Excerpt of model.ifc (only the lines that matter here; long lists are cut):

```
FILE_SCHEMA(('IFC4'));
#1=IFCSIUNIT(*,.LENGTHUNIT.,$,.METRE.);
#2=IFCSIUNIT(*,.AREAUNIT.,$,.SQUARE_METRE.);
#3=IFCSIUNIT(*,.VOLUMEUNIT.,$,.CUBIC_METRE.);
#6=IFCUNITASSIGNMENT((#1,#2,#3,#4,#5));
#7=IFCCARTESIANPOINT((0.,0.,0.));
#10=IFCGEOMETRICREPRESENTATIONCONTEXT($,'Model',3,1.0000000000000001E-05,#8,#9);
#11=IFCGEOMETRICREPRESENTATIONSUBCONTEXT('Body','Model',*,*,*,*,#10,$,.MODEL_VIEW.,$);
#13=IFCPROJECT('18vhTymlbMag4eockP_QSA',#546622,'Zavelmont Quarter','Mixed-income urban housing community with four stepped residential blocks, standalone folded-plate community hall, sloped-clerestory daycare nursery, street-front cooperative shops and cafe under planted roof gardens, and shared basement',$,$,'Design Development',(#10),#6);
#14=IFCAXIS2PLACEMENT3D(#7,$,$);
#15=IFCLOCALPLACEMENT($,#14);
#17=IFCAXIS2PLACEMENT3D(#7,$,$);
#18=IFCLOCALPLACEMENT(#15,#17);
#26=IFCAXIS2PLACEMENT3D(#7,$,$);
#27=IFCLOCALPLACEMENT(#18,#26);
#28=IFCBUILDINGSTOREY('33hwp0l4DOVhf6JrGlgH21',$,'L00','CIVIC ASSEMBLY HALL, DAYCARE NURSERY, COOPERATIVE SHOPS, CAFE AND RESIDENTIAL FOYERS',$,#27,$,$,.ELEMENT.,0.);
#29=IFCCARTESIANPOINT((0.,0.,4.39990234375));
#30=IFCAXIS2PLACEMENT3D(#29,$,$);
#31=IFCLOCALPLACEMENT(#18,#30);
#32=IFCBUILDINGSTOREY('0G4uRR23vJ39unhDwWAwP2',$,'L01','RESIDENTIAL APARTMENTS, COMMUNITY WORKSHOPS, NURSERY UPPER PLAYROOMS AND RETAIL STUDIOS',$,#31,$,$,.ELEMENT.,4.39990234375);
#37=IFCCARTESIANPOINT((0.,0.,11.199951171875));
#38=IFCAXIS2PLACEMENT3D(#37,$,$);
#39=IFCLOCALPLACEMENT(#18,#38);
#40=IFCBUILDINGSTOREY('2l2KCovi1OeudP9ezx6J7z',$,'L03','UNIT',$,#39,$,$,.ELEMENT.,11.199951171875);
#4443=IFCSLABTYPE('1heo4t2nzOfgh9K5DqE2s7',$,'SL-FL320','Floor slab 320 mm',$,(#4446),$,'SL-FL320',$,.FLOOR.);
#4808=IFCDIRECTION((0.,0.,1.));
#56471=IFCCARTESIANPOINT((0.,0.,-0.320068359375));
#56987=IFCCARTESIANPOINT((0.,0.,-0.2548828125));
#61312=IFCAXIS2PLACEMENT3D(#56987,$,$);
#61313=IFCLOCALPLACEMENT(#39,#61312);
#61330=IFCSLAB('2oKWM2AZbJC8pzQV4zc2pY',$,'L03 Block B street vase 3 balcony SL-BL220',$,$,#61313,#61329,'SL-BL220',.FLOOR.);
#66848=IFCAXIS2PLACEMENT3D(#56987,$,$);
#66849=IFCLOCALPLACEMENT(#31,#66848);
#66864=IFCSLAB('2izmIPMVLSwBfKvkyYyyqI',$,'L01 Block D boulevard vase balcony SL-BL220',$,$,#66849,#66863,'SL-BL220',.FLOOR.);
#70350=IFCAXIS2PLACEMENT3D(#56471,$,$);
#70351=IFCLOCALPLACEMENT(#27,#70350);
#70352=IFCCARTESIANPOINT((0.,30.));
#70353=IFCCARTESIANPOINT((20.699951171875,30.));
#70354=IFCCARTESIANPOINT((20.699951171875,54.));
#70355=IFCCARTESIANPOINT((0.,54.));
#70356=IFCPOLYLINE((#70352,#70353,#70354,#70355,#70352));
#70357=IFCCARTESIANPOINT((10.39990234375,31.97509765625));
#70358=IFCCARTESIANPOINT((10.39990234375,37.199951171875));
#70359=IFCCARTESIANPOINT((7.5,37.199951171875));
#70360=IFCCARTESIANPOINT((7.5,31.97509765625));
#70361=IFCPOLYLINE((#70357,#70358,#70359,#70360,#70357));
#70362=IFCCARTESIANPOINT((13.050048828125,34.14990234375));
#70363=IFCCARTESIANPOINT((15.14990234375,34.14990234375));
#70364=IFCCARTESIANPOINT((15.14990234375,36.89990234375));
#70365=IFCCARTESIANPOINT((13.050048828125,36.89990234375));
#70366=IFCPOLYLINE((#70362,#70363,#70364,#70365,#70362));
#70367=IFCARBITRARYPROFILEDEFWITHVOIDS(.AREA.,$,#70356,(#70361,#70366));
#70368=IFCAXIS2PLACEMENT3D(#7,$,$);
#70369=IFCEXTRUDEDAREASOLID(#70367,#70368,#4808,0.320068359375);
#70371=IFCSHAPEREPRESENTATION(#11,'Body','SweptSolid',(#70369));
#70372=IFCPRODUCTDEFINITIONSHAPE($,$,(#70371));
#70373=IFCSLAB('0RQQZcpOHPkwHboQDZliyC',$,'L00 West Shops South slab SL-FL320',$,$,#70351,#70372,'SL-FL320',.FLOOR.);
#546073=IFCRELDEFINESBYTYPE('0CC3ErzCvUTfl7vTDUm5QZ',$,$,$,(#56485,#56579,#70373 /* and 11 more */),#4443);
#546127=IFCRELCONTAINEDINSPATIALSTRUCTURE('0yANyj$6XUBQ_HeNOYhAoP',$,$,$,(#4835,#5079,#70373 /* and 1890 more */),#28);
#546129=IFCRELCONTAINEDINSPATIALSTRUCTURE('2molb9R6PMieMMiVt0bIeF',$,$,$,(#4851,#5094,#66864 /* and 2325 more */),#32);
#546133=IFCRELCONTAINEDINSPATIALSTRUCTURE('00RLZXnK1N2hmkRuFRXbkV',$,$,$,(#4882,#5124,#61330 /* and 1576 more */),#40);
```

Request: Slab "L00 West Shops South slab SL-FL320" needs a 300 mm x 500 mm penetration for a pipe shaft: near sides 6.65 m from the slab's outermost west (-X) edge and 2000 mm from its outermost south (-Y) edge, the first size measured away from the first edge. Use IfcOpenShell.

```python
import numpy as np
import ifcopenshell
import ifcopenshell.api.feature
import ifcopenshell.api.geometry
import ifcopenshell.api.root
import ifcopenshell.geom
import ifcopenshell.util.placement
import ifcopenshell.util.representation
import ifcopenshell.util.shape
import ifcopenshell.util.unit

model = ifcopenshell.open("model.ifc")
unit_scale = ifcopenshell.util.unit.calculate_unit_scale(model)
settings = ifcopenshell.geom.settings()


def volume(element):
    """Net volume in cubic metres, openings subtracted."""
    shape = ifcopenshell.geom.create_shape(settings, element)
    return ifcopenshell.util.shape.get_volume(shape.geometry)


slab = model.by_guid("0RQQZcpOHPkwHboQDZliyC")
before = volume(slab)

# Extent in the slab's own axes, in metres. The edges named are its -X and -Y sides.
slab_shape = ifcopenshell.geom.create_shape(settings, slab)
vertices = ifcopenshell.util.shape.get_vertices(slab_shape.geometry)
x_min, y_min, bottom = vertices.min(axis=0)
top = vertices[:, 2].max()

opening = ifcopenshell.api.root.create_entity(model, ifc_class="IfcOpeningElement", name="Pipe shaft opening", predefined_type="OPENING")
context = ifcopenshell.util.representation.get_context(model, "Model", "Body", "MODEL_VIEW")
width, depth = 0.3, 0.5
outline = [(0.0, 0.0), (width, 0.0), (width, depth), (0.0, depth), (0.0, 0.0)]
# Overshoot both faces by 50 mm so the cut is clean.
shape = ifcopenshell.api.geometry.add_slab_representation(
    model, context=context, depth=top - bottom + 0.1, polyline=outline
)
ifcopenshell.api.geometry.assign_representation(model, product=opening, representation=shape)

matrix = ifcopenshell.util.placement.get_local_placement(slab.ObjectPlacement)
matrix[:, 3] = matrix @ np.append(np.array([x_min + 6.65, y_min + 2, bottom - 0.05]) / unit_scale, 1.0)
ifcopenshell.api.geometry.edit_object_placement(model, product=opening, matrix=matrix, is_si=False)
ifcopenshell.api.feature.add_feature(model, feature=opening, element=slab)

after = volume(slab)

print(f"slab volume {before:.3f} -> {after:.3f} m3")

model.write("model_v2.ifc")
```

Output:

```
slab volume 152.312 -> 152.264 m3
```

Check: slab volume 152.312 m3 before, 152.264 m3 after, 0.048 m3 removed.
